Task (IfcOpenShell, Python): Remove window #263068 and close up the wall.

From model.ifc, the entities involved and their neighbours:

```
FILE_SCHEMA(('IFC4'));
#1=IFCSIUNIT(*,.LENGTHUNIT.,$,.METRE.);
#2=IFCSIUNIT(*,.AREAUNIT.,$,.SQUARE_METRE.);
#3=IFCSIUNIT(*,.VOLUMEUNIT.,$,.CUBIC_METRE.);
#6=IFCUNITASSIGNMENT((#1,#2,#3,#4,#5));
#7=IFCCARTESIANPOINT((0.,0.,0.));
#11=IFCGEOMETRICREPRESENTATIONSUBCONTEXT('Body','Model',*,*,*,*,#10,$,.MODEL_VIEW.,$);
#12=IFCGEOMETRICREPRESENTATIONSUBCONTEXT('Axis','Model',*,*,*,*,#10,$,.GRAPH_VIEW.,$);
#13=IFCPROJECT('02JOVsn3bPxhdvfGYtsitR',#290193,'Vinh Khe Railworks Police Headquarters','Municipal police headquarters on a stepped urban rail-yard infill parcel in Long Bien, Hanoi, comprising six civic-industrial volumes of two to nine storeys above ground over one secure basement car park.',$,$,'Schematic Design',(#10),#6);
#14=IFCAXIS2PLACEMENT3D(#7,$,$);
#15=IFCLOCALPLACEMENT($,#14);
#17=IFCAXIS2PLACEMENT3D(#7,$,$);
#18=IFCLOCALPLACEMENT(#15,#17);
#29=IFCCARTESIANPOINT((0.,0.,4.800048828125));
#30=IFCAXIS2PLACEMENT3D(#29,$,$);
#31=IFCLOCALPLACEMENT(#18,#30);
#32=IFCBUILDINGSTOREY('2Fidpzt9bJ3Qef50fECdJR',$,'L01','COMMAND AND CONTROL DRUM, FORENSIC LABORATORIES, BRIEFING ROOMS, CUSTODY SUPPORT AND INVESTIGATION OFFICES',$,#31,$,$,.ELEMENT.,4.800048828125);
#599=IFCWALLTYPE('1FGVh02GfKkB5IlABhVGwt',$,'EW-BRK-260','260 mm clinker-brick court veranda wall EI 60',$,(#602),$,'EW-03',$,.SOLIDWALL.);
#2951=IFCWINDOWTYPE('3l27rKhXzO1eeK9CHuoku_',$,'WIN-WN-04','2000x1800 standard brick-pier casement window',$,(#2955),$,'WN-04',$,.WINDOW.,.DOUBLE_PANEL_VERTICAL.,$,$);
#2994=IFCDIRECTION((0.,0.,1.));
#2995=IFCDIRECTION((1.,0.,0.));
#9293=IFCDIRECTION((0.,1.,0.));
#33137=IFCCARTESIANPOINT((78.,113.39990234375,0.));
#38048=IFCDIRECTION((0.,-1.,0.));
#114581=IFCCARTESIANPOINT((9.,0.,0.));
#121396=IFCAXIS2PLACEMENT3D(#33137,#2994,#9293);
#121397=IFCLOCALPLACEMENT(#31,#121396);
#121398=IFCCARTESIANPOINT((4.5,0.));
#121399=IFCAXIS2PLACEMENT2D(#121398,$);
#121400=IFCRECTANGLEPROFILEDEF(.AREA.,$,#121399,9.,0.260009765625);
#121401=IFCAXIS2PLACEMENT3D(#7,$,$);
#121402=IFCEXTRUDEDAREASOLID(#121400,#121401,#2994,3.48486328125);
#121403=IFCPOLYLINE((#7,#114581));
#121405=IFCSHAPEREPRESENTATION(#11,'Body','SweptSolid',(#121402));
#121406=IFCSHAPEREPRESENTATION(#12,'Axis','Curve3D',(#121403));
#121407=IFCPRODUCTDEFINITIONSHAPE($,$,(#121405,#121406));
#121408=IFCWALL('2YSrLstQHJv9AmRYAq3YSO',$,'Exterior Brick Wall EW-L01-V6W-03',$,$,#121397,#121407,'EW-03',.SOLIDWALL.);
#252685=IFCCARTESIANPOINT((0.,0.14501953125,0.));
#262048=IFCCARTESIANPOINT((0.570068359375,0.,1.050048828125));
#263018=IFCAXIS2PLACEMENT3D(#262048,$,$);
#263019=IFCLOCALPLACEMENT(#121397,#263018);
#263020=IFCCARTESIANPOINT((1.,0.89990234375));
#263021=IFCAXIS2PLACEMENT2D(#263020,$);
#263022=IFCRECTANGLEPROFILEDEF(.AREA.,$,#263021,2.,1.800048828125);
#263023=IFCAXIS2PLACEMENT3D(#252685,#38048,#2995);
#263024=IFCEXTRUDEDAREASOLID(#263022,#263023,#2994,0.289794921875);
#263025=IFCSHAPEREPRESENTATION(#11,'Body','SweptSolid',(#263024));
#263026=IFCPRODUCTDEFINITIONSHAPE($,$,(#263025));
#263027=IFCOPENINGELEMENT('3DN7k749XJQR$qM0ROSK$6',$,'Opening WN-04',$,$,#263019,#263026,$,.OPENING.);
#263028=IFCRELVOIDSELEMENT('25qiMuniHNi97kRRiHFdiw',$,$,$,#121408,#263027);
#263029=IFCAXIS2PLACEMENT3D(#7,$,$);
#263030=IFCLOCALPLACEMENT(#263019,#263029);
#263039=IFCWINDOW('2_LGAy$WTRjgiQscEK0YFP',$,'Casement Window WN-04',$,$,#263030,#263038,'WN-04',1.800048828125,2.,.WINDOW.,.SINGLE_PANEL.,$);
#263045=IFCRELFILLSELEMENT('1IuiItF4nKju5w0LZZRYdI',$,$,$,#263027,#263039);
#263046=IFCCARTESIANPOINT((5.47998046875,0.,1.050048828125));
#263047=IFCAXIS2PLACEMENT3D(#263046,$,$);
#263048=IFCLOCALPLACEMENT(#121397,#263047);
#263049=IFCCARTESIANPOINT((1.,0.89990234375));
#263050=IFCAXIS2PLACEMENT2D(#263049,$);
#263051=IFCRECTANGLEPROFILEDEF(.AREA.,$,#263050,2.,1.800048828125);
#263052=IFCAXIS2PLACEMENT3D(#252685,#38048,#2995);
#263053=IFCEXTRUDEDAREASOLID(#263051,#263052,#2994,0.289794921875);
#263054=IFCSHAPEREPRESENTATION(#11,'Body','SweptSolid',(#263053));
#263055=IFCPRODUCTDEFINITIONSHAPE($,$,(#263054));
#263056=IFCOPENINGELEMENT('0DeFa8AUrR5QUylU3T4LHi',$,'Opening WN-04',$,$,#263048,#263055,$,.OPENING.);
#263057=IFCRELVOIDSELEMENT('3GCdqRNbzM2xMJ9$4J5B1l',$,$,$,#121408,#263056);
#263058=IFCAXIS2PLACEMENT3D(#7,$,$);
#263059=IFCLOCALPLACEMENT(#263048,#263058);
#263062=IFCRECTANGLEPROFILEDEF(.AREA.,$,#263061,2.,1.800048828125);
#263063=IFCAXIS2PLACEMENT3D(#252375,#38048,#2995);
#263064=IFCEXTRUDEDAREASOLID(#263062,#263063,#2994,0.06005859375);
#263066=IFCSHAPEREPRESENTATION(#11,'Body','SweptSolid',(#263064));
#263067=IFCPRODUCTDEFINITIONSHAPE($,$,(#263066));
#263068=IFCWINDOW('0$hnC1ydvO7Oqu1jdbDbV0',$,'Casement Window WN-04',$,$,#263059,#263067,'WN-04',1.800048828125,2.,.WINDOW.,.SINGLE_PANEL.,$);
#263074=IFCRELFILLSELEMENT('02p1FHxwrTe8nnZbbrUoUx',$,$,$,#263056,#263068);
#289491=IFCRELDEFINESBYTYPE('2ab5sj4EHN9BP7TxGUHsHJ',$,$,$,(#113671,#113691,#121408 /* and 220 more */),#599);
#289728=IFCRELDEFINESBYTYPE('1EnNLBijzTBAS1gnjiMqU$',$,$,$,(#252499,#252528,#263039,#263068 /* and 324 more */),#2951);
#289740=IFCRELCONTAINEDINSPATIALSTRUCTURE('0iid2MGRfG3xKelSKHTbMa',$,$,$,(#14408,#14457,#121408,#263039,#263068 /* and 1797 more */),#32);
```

```python
import ifcopenshell
import ifcopenshell.api.feature
import ifcopenshell.api.root
import ifcopenshell.geom
import ifcopenshell.util.shape

model = ifcopenshell.open("model.ifc")
settings = ifcopenshell.geom.settings()


def volume(element):
    """Net volume in cubic metres, openings subtracted."""
    shape = ifcopenshell.geom.create_shape(settings, element)
    return ifcopenshell.util.shape.get_volume(shape.geometry)


window = model.by_guid("0$hnC1ydvO7Oqu1jdbDbV0")
opening = window.FillsVoids[0].RelatingOpeningElement
wall = opening.VoidsElements[0].RelatingBuildingElement
before = volume(wall)

ifcopenshell.api.root.remove_product(model, product=window)
ifcopenshell.api.feature.remove_feature(model, feature=opening)

after = volume(wall)

print(f"wall volume {before:.3f} -> {after:.3f} m3")

model.write("model_v2.ifc")
```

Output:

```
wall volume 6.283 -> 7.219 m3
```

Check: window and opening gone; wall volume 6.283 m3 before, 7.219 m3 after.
